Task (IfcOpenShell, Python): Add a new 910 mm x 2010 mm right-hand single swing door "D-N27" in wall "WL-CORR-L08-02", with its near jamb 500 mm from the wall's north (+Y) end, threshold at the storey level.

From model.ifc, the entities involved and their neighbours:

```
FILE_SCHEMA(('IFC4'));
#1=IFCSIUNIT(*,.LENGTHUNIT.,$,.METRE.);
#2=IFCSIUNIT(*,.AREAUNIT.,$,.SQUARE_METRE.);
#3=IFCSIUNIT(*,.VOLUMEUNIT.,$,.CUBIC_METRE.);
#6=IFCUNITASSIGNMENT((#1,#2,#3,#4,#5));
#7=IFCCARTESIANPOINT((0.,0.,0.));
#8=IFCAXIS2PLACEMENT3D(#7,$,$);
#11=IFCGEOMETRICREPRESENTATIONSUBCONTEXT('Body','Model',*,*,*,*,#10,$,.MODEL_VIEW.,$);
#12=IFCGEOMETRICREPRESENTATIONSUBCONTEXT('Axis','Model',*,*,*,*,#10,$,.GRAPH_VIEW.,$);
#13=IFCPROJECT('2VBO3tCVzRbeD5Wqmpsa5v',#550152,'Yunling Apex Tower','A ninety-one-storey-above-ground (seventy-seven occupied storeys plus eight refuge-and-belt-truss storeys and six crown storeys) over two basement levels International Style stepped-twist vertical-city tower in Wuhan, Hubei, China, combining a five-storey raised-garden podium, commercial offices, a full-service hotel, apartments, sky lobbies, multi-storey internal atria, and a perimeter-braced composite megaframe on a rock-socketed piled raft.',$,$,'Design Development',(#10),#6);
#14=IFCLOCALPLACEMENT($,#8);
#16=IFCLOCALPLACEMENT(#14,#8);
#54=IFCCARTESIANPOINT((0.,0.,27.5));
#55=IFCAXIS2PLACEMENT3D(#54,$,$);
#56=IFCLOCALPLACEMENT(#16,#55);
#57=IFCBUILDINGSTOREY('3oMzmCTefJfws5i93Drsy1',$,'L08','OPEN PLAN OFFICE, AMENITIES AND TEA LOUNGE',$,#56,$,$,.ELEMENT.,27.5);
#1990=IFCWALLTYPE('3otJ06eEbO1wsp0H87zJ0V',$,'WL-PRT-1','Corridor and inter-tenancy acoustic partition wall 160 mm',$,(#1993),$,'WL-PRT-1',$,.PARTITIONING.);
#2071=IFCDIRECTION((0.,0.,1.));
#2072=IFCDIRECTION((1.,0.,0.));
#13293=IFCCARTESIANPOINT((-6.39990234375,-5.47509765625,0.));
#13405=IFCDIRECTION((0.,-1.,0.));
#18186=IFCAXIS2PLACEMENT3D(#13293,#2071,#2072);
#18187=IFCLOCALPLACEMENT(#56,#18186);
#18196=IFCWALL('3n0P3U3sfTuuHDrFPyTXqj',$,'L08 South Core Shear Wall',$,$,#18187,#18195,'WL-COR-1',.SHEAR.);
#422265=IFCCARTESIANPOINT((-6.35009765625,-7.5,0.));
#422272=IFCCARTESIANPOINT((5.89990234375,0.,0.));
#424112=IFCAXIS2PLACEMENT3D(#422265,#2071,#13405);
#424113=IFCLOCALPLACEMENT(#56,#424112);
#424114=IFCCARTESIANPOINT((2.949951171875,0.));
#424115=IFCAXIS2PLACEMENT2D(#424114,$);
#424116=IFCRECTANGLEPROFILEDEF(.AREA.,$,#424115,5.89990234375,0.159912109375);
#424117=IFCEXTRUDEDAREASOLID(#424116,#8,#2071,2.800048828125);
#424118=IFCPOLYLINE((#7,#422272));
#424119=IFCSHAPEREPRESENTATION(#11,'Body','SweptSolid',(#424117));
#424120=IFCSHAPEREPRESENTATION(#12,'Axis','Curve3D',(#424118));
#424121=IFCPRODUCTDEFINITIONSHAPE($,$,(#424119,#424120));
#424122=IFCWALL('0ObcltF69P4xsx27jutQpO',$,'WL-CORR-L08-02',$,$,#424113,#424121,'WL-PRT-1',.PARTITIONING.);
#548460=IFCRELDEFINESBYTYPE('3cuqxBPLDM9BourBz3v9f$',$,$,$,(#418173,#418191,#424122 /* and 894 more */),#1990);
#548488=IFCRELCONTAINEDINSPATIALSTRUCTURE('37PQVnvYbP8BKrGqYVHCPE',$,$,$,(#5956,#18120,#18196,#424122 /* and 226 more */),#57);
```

```python
import numpy as np
import ifcopenshell
import ifcopenshell.api.feature
import ifcopenshell.api.geometry
import ifcopenshell.api.root
import ifcopenshell.api.spatial
import ifcopenshell.geom
import ifcopenshell.util.element
import ifcopenshell.util.placement
import ifcopenshell.util.representation
import ifcopenshell.util.shape
import ifcopenshell.util.unit

model = ifcopenshell.open("model.ifc")
unit_scale = ifcopenshell.util.unit.calculate_unit_scale(model)
settings = ifcopenshell.geom.settings()


def volume(element):
    """Net volume in cubic metres, openings subtracted."""
    shape = ifcopenshell.geom.create_shape(settings, element)
    return ifcopenshell.util.shape.get_volume(shape.geometry)


wall = model.by_id(424122)
storey = ifcopenshell.util.element.get_container(wall, ifc_class="IfcBuildingStorey")
context = ifcopenshell.util.representation.get_context(model, "Model", "Body", "MODEL_VIEW")
before = volume(wall)

width, height, from_end, sill = 0.91, 2.01, 0.5, 0.0  # metres

# The wall runs along its own X axis, and the end named is its -X end.
wall_shape = ifcopenshell.geom.create_shape(settings, wall)
x, y, z = ifcopenshell.util.shape.get_vertices(wall_shape.geometry).T
start = x.min() + from_end
face, thickness = float(y.min()), float(y.max() - y.min())
wall_matrix = ifcopenshell.util.placement.get_local_placement(wall.ObjectPlacement)
level = ifcopenshell.util.placement.get_local_placement(storey.ObjectPlacement)[2, 3]


def in_wall(x, y):
    """Placement at x, y metres in the wall's axes, at sill height."""
    matrix = wall_matrix.copy()
    matrix[:, 3] = wall_matrix @ np.array([x / unit_scale, y / unit_scale, 0.0, 1.0])
    matrix[2, 3] = level + sill / unit_scale
    return matrix


# Opening: a box that overshoots both wall faces by 50 mm.
opening = ifcopenshell.api.root.create_entity(model, ifc_class="IfcOpeningElement", predefined_type="OPENING")
box = ifcopenshell.api.geometry.add_wall_representation(
    model, context=context, length=width, height=height, thickness=thickness + 0.1
)
ifcopenshell.api.geometry.assign_representation(model, product=opening, representation=box)
ifcopenshell.api.geometry.edit_object_placement(model, product=opening, matrix=in_wall(start, face - 0.05), is_si=False)
ifcopenshell.api.feature.add_feature(model, feature=opening, element=wall)

door = ifcopenshell.api.root.create_entity(model, ifc_class="IfcDoor", name="D-N27", predefined_type="DOOR")
door.OverallWidth, door.OverallHeight = width / unit_scale, height / unit_scale
door.OperationType = "SINGLE_SWING_RIGHT"
body = ifcopenshell.api.geometry.add_door_representation(
    model,
    context=context,
    overall_width=door.OverallWidth,
    overall_height=door.OverallHeight,
    operation_type="SINGLE_SWING_RIGHT",
    lining_properties={"LiningDepth": thickness / unit_scale, "ThresholdDepth": thickness / unit_scale},
)
ifcopenshell.api.geometry.assign_representation(model, product=door, representation=body)
ifcopenshell.api.spatial.assign_container(model, products=[door], relating_structure=storey)
ifcopenshell.api.feature.add_filling(model, opening=opening, element=door)

# The lining spans the wall, so the door starts at the wall face.
ifcopenshell.api.geometry.edit_object_placement(model, product=door, matrix=in_wall(start, face), is_si=False)

after = volume(wall)

print(f"wall volume {before:.3f} -> {after:.3f} m3")

model.write("model_rev.ifc")
```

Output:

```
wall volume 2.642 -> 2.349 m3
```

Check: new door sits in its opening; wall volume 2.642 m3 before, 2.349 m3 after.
